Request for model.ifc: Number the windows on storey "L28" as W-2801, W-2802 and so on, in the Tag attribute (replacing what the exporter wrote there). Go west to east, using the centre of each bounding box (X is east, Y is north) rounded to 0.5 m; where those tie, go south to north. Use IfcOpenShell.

First a look at what the model holds.

```python
import ifcopenshell
import ifcopenshell.util.element
import ifcopenshell.util.placement

model = ifcopenshell.open("model.ifc")
print(model.schema)
storey = next(s for s in model.by_type("IfcBuildingStorey") if s.Name == "L28")
windows = [e for e in ifcopenshell.util.element.get_decomposition(storey) if e.is_a("IfcWindow")]
for e in sorted(windows, key=lambda e: e.id()):
    origin = ifcopenshell.util.placement.get_local_placement(e.ObjectPlacement)[:3, 3]
    print(e.id(), e.Tag, e.Name, origin.round(2) + 0.0, sep=" | ")
```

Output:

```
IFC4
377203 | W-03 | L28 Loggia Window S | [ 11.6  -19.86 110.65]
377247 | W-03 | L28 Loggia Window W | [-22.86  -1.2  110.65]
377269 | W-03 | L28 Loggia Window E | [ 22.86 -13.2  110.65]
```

```python
import ifcopenshell
import ifcopenshell.geom
import ifcopenshell.util.element
import ifcopenshell.util.shape

model = ifcopenshell.open("model.ifc")
settings = ifcopenshell.geom.settings()
settings.set("use-world-coords", True)


def centre(element):
    shape = ifcopenshell.geom.create_shape(settings, element)
    return ifcopenshell.util.shape.get_bbox_centroid(shape.geometry)


storey = next(s for s in model.by_type("IfcBuildingStorey") if s.Name == "L28")
windows = [e for e in ifcopenshell.util.element.get_decomposition(storey) if e.is_a("IfcWindow")]

# Insertion points can sit at a corner or the storey origin, so sort by the geometry (in metres).
centres = {e: centre(e) for e in windows}
windows.sort(key=lambda e: (round(centres[e][0] / 0.5), centres[e][1]))

for i, e in enumerate(windows, start=1):
    number = f"W-28{i:02d}"
    e.Tag = number
    print(e.id(), number)

model.write("model_rev.ifc")
```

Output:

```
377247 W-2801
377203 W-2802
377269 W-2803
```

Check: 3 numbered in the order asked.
